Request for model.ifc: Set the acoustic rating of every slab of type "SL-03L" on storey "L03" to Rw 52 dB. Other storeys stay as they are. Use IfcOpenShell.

First a look at what the model holds.

```python
import ifcopenshell
import ifcopenshell.util.element

model = ifcopenshell.open("model.ifc")
print(model.schema)
storey = next(s for s in model.by_type("IfcBuildingStorey") if s.Name == "L03")
slabs = [e for e in ifcopenshell.util.element.get_decomposition(storey) if e.is_a("IfcSlab")]
seen = {}
for e in slabs:
    element_type = ifcopenshell.util.element.get_type(e)
    key = (element_type.Name if element_type != e and element_type else None, ifcopenshell.util.element.get_pset(e, "Pset_SlabCommon", "AcousticRating"))
    seen[key] = seen.get(key, 0) + 1
for (name, value), count in sorted(seen.items(), key=str):
    print(count, "x", name, "|", value)
```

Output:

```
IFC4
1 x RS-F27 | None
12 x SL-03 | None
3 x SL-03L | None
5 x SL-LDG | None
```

```python
import ifcopenshell
import ifcopenshell.api.pset
import ifcopenshell.util.element

model = ifcopenshell.open("model.ifc")

storey = next(s for s in model.by_type("IfcBuildingStorey") if s.Name == "L03")
slabs = [e for e in ifcopenshell.util.element.get_decomposition(storey) if e.is_a("IfcSlab")]

count = 0
for e in slabs:
    element_type = ifcopenshell.util.element.get_type(e)
    if element_type in (None, e) or element_type.Name != "SL-03L":
        continue
    # add_pset returns the element's existing set when there is one.
    pset = ifcopenshell.api.pset.add_pset(model, product=e, name="Pset_SlabCommon")
    ifcopenshell.api.pset.edit_pset(model, pset=pset, properties={"AcousticRating": "Rw 52 dB"})
    count += 1

print(count, "slabs updated")

model.write("model_rev.ifc")
```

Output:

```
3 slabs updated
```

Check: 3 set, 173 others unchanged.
